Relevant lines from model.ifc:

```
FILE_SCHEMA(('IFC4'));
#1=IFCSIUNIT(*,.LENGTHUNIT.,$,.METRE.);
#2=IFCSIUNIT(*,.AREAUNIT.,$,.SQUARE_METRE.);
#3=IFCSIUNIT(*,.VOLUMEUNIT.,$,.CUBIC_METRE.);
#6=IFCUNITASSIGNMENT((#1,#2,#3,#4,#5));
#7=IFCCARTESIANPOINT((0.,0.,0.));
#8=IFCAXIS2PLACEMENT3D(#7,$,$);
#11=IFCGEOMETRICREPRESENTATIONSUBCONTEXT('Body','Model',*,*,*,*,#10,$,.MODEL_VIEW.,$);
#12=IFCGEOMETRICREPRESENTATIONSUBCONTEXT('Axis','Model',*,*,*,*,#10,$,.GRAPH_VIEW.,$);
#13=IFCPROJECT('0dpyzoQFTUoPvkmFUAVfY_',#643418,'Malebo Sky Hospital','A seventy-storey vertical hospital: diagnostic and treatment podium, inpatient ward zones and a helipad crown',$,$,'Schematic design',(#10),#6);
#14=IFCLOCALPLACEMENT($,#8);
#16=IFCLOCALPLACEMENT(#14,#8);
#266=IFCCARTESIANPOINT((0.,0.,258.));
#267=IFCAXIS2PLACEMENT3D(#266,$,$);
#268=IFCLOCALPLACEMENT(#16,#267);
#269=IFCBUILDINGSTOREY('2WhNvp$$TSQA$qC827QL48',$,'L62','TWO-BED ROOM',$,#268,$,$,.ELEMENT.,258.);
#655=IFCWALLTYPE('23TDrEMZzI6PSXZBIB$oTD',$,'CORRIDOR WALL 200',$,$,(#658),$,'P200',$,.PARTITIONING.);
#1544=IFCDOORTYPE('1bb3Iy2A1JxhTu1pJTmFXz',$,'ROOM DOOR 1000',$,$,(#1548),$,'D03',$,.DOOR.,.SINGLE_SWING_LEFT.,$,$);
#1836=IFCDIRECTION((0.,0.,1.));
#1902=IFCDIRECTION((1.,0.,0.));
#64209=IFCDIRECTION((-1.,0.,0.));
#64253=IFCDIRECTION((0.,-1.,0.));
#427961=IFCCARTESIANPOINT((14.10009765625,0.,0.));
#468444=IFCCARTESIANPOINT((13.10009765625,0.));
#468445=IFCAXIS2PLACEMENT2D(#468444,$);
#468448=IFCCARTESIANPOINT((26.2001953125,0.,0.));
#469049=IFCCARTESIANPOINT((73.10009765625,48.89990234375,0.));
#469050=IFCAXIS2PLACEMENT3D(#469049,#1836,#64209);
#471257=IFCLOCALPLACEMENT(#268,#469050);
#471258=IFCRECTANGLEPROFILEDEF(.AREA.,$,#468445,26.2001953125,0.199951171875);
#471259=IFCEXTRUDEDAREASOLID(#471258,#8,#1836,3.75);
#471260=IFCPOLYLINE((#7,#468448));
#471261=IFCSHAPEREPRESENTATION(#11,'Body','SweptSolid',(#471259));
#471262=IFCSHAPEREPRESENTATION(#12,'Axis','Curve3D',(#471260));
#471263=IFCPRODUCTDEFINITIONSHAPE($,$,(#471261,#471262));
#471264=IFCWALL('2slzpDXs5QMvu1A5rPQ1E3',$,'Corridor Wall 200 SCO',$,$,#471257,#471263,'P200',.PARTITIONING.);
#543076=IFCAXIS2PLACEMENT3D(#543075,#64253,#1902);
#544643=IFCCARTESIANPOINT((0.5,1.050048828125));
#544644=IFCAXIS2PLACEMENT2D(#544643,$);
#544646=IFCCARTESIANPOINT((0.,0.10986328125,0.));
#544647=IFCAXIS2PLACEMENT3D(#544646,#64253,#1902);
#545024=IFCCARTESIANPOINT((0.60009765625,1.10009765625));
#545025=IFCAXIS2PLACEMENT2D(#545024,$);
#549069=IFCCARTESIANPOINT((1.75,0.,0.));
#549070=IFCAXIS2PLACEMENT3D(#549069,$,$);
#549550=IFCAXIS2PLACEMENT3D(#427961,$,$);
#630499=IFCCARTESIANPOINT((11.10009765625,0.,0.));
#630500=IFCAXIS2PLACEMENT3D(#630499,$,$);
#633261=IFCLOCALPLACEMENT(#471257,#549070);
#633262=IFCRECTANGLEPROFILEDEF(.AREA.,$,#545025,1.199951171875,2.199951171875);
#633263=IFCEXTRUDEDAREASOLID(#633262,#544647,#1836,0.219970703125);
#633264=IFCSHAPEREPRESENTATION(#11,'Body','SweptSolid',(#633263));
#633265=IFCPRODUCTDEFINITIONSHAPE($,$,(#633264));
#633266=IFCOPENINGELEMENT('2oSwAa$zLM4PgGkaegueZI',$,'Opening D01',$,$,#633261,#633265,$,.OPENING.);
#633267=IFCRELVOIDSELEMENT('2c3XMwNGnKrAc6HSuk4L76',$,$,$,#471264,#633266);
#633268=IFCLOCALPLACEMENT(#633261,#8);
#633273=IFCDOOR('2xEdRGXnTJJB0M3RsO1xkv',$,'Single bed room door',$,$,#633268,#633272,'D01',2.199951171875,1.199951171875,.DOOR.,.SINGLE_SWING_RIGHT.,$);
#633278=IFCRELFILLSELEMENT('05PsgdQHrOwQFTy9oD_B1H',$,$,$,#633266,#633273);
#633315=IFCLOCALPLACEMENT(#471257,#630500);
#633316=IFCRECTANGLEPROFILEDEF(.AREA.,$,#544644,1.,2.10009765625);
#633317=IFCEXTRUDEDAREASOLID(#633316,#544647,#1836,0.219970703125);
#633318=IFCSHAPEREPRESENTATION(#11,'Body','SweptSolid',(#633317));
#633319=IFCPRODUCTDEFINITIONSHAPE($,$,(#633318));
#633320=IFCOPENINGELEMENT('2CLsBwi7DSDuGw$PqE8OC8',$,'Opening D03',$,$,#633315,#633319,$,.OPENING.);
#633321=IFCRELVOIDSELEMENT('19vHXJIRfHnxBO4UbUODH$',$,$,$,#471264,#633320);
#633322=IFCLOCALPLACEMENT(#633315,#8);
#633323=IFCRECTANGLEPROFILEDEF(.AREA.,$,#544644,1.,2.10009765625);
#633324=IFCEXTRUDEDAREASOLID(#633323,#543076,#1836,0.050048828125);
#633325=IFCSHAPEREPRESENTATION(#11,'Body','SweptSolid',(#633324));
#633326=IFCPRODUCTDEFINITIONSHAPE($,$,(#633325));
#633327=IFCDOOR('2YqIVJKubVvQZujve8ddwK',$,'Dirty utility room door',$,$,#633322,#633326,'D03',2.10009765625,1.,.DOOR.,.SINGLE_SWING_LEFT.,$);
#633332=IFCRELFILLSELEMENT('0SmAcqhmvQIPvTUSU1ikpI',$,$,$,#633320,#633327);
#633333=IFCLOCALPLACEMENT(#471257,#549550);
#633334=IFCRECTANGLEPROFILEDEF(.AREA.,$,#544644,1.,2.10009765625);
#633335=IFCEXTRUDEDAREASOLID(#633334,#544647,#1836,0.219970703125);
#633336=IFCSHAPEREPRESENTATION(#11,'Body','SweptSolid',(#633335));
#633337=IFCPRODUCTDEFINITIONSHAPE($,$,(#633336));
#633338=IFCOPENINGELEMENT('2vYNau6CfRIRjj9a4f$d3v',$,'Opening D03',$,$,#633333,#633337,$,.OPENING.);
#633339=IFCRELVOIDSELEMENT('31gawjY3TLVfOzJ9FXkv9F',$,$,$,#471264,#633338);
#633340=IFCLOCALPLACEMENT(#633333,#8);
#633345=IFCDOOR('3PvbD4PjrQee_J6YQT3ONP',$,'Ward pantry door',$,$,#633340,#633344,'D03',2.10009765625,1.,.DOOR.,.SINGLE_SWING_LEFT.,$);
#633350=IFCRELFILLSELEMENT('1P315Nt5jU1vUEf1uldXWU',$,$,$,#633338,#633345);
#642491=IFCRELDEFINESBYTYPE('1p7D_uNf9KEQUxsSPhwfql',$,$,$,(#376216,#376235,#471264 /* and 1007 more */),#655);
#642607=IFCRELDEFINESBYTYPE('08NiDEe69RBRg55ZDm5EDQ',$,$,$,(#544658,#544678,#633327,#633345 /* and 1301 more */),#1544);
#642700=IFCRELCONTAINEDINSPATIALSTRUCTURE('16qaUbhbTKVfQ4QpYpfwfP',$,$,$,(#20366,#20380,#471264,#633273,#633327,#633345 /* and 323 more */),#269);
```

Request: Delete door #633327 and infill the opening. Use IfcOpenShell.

```python
import ifcopenshell
import ifcopenshell.api.feature
import ifcopenshell.api.root
import ifcopenshell.geom
import ifcopenshell.util.shape

model = ifcopenshell.open("model.ifc")
settings = ifcopenshell.geom.settings()


def volume(element):
    """Net volume in cubic metres, openings subtracted."""
    shape = ifcopenshell.geom.create_shape(settings, element)
    return ifcopenshell.util.shape.get_volume(shape.geometry)


door = model.by_guid("2YqIVJKubVvQZujve8ddwK")
opening = door.FillsVoids[0].RelatingOpeningElement
wall = opening.VoidsElements[0].RelatingBuildingElement
before = volume(wall)

ifcopenshell.api.root.remove_product(model, product=door)
ifcopenshell.api.feature.remove_feature(model, feature=opening)

after = volume(wall)

print(f"wall volume {before:.3f} -> {after:.3f} m3")

model.write("model_v2.ifc")
```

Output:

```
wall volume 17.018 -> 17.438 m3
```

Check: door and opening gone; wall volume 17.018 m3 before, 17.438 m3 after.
